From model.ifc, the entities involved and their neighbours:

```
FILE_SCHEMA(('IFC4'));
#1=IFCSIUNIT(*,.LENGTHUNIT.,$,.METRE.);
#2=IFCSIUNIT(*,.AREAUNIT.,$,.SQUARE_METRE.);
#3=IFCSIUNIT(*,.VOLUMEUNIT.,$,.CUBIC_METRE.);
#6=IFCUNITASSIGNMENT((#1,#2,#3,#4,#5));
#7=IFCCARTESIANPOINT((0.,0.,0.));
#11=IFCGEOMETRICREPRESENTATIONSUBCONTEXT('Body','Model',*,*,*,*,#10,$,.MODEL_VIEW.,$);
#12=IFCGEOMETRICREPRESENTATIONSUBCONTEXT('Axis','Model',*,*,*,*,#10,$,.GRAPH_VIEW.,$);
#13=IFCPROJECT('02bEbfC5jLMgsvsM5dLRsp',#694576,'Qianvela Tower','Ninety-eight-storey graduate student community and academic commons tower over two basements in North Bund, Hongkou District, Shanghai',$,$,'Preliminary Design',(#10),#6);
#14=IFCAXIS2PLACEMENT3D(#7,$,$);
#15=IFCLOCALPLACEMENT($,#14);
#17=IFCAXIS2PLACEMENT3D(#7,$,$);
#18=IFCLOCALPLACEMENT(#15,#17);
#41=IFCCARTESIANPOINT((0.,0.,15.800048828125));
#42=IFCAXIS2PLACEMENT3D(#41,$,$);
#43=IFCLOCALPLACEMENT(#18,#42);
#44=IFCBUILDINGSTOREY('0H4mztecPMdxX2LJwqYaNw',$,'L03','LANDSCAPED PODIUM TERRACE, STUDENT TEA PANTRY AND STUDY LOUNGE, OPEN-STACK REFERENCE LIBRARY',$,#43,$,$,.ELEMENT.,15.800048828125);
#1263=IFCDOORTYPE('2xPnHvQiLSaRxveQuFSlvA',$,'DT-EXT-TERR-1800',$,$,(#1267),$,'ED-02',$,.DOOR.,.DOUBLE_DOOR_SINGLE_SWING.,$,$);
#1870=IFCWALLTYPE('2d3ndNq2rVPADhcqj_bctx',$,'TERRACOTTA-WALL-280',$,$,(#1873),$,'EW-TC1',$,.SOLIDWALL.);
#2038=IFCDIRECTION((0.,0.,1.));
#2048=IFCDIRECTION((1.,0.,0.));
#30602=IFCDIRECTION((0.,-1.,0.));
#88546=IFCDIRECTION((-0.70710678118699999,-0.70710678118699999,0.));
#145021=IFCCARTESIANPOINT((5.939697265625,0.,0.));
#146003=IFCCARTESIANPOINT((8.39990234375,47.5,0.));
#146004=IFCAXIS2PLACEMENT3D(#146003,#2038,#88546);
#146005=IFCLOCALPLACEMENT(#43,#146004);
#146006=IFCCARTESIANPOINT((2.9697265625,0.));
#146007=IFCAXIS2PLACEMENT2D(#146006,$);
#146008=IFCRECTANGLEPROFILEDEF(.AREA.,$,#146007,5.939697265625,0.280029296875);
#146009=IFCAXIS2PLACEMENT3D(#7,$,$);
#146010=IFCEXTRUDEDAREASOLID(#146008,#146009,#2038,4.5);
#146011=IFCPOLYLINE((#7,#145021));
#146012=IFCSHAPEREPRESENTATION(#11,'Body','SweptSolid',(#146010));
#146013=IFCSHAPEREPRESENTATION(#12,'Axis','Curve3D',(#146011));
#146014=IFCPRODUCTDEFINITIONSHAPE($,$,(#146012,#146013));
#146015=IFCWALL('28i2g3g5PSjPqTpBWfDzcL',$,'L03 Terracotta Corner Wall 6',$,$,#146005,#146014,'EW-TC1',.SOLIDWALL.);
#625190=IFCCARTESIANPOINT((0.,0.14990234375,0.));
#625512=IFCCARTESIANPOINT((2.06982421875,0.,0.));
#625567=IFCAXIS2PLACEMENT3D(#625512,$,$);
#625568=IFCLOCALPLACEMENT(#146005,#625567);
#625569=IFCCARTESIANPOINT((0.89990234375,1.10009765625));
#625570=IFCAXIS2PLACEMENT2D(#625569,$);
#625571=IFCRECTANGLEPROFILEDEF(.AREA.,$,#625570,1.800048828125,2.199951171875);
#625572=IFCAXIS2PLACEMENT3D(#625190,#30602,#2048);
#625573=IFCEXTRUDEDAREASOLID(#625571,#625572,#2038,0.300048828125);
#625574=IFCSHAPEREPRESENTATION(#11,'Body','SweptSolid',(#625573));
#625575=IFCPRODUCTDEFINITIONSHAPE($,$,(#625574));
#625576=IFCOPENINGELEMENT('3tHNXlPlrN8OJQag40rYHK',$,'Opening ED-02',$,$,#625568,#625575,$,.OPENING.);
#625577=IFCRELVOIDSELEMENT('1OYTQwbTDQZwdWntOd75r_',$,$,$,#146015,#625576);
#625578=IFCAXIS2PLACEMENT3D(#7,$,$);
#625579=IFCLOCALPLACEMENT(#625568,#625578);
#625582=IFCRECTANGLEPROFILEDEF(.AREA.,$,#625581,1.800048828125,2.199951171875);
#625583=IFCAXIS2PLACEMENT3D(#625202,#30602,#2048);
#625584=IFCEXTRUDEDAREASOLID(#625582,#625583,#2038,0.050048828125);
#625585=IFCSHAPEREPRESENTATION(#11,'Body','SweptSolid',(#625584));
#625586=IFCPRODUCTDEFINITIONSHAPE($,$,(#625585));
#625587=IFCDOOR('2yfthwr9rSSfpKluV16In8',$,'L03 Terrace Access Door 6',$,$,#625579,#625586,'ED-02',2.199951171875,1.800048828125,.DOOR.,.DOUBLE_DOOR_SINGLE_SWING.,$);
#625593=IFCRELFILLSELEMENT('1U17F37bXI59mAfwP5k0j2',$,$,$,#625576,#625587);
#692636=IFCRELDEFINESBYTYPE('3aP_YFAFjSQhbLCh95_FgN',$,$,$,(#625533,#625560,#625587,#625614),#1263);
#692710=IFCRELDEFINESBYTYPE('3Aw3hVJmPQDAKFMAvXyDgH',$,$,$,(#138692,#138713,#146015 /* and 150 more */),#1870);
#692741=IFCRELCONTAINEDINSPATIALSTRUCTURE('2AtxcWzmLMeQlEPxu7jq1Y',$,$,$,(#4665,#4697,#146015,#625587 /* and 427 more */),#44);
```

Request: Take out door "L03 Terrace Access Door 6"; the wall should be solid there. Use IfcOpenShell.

```python
import ifcopenshell
import ifcopenshell.api.feature
import ifcopenshell.api.root
import ifcopenshell.geom
import ifcopenshell.util.shape

model = ifcopenshell.open("model.ifc")
settings = ifcopenshell.geom.settings()


def volume(element):
    """Net volume in cubic metres, openings subtracted."""
    shape = ifcopenshell.geom.create_shape(settings, element)
    return ifcopenshell.util.shape.get_volume(shape.geometry)


door = model.by_guid("2yfthwr9rSSfpKluV16In8")
opening = door.FillsVoids[0].RelatingOpeningElement
wall = opening.VoidsElements[0].RelatingBuildingElement
before = volume(wall)

ifcopenshell.api.root.remove_product(model, product=door)
ifcopenshell.api.feature.remove_feature(model, feature=opening)

after = volume(wall)

print(f"wall volume {before:.3f} -> {after:.3f} m3")

model.write("model-out.ifc")
```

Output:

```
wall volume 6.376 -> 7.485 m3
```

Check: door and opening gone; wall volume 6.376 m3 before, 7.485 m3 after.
